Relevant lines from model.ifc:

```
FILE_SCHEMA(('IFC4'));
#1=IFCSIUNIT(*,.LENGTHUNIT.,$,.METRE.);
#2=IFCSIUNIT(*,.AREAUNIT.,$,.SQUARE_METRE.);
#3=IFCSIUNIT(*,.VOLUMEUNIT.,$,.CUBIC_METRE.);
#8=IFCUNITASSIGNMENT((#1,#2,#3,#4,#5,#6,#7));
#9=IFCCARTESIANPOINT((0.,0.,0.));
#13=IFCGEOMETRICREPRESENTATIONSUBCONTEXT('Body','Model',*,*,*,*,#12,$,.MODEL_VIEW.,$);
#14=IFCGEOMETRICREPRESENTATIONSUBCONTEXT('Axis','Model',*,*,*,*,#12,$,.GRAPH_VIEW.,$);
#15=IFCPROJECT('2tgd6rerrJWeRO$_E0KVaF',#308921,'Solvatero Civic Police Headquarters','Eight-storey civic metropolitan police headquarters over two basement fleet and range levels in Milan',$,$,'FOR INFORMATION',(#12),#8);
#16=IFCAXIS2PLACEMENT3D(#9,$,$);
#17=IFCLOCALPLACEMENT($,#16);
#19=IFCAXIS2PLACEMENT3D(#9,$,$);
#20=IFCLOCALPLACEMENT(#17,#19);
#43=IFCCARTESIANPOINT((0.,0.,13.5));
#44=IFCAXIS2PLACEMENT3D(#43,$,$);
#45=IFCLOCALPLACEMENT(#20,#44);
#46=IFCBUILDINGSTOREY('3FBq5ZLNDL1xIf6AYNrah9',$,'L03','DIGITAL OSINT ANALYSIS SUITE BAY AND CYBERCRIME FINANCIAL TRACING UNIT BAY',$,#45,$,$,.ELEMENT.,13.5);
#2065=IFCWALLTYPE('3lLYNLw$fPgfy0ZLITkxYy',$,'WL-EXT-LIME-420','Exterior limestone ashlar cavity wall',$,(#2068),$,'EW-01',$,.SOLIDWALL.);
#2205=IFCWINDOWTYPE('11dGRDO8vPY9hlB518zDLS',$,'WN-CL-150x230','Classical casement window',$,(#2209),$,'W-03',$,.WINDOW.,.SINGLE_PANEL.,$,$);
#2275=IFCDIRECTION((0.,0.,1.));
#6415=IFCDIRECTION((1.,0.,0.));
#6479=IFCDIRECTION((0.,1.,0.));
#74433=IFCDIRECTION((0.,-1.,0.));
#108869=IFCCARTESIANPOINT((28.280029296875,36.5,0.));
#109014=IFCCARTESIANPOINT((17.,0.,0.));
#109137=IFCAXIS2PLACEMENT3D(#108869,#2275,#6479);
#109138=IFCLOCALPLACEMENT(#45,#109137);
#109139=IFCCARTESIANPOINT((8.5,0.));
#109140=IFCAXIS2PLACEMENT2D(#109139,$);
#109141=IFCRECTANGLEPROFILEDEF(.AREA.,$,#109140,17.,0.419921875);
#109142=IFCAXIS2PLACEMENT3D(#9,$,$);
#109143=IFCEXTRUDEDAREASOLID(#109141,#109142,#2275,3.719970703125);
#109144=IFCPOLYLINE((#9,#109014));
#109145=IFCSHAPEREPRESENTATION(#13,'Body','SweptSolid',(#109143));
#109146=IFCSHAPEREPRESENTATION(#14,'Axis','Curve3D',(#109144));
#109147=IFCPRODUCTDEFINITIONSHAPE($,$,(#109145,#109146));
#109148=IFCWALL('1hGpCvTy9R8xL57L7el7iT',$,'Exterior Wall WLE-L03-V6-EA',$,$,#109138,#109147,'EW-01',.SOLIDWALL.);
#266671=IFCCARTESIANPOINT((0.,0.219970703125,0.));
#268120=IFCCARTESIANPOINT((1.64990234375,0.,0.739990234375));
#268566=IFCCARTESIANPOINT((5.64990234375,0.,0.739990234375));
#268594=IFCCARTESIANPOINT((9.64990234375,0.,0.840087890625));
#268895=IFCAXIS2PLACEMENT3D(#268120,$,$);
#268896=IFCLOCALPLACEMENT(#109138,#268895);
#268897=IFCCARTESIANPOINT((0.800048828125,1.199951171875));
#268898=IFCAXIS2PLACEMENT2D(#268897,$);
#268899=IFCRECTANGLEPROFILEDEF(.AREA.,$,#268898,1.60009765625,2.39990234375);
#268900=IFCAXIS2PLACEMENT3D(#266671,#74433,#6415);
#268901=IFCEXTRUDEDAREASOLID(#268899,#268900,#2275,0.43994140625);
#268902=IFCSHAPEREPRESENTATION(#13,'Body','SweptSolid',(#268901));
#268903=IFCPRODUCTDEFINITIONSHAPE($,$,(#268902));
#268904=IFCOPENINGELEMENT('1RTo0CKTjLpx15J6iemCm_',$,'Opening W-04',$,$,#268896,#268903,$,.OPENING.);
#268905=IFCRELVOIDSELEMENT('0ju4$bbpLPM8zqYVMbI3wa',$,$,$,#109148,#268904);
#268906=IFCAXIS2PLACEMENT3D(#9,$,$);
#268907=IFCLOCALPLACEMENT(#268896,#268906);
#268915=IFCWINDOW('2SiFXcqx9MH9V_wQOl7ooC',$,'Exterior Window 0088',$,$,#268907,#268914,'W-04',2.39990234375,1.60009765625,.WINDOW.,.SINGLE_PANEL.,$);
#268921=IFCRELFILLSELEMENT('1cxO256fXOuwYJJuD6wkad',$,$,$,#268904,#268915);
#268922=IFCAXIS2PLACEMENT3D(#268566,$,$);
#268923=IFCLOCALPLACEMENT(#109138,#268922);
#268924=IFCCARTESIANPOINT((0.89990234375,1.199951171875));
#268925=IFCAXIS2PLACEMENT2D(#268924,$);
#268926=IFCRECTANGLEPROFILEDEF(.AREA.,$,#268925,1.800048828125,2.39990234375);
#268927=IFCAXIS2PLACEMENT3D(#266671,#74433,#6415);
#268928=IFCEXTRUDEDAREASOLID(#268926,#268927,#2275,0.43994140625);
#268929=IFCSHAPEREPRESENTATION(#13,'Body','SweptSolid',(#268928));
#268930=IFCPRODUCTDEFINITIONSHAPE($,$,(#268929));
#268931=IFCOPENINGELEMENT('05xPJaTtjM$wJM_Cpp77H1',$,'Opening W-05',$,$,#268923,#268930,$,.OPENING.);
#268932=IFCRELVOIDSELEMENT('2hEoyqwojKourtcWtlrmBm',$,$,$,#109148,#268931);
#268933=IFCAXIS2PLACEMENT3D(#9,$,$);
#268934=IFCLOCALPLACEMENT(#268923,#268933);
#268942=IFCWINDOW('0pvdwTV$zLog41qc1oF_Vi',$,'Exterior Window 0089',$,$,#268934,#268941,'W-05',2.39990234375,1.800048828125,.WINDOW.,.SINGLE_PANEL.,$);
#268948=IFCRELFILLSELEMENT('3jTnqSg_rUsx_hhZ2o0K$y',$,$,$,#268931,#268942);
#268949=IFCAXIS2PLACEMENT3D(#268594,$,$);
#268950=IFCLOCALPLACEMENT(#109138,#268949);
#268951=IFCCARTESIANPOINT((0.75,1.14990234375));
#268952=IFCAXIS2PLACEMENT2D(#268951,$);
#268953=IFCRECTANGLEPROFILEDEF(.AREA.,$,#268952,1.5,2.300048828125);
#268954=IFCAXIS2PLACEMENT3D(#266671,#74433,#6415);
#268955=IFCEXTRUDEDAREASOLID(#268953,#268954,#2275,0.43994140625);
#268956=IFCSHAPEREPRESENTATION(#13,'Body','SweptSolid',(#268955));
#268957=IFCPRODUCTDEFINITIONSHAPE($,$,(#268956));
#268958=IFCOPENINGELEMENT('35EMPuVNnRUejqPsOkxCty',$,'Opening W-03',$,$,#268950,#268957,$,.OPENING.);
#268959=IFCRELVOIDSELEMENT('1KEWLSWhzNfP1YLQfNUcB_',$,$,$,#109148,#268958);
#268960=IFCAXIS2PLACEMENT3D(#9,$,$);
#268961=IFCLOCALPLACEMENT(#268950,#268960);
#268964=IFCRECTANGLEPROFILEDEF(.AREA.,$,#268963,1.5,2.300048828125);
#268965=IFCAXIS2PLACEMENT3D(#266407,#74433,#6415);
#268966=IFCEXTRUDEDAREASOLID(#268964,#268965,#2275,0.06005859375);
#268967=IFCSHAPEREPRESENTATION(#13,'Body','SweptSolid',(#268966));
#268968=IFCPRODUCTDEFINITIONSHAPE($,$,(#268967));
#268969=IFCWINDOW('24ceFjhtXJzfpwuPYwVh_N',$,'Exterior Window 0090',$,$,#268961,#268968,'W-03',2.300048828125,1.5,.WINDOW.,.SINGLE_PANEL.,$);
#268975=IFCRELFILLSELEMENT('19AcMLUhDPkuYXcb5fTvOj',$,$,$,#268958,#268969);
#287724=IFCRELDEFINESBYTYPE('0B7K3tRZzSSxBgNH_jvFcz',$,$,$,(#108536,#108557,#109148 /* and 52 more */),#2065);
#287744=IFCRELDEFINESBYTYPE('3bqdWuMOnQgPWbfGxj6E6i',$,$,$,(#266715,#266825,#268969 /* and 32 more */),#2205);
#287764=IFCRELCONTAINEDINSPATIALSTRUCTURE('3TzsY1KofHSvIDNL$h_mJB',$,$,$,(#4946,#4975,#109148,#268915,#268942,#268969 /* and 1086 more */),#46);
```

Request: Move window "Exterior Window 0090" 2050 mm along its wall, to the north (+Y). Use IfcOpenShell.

```python
import ifcopenshell
import ifcopenshell.api.geometry
import ifcopenshell.util.placement
import ifcopenshell.util.unit

model = ifcopenshell.open("model.ifc")
unit_scale = ifcopenshell.util.unit.calculate_unit_scale(model)

window = model.by_id(268969)
opening = window.FillsVoids[0].RelatingOpeningElement
wall = opening.VoidsElements[0].RelatingBuildingElement

wall_matrix = ifcopenshell.util.placement.get_local_placement(wall.ObjectPlacement)
shift = wall_matrix[:3, 0] * 2.05 / unit_scale
before = ifcopenshell.util.placement.get_local_placement(window.ObjectPlacement)[:3, 3].copy()

# The window is placed relative to its opening, so it follows when the opening moves.
matrix = ifcopenshell.util.placement.get_local_placement(opening.ObjectPlacement)
matrix[:3, 3] += shift
ifcopenshell.api.geometry.edit_object_placement(
    model, product=opening, matrix=matrix, is_si=False, should_transform_children=True
)

after = ifcopenshell.util.placement.get_local_placement(window.ObjectPlacement)[:3, 3]
print("window moved by", (after - before).round(3) + 0.0)

model.write("model-out.ifc")
```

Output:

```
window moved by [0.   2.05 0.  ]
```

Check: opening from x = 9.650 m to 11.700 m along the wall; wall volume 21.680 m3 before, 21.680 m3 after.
